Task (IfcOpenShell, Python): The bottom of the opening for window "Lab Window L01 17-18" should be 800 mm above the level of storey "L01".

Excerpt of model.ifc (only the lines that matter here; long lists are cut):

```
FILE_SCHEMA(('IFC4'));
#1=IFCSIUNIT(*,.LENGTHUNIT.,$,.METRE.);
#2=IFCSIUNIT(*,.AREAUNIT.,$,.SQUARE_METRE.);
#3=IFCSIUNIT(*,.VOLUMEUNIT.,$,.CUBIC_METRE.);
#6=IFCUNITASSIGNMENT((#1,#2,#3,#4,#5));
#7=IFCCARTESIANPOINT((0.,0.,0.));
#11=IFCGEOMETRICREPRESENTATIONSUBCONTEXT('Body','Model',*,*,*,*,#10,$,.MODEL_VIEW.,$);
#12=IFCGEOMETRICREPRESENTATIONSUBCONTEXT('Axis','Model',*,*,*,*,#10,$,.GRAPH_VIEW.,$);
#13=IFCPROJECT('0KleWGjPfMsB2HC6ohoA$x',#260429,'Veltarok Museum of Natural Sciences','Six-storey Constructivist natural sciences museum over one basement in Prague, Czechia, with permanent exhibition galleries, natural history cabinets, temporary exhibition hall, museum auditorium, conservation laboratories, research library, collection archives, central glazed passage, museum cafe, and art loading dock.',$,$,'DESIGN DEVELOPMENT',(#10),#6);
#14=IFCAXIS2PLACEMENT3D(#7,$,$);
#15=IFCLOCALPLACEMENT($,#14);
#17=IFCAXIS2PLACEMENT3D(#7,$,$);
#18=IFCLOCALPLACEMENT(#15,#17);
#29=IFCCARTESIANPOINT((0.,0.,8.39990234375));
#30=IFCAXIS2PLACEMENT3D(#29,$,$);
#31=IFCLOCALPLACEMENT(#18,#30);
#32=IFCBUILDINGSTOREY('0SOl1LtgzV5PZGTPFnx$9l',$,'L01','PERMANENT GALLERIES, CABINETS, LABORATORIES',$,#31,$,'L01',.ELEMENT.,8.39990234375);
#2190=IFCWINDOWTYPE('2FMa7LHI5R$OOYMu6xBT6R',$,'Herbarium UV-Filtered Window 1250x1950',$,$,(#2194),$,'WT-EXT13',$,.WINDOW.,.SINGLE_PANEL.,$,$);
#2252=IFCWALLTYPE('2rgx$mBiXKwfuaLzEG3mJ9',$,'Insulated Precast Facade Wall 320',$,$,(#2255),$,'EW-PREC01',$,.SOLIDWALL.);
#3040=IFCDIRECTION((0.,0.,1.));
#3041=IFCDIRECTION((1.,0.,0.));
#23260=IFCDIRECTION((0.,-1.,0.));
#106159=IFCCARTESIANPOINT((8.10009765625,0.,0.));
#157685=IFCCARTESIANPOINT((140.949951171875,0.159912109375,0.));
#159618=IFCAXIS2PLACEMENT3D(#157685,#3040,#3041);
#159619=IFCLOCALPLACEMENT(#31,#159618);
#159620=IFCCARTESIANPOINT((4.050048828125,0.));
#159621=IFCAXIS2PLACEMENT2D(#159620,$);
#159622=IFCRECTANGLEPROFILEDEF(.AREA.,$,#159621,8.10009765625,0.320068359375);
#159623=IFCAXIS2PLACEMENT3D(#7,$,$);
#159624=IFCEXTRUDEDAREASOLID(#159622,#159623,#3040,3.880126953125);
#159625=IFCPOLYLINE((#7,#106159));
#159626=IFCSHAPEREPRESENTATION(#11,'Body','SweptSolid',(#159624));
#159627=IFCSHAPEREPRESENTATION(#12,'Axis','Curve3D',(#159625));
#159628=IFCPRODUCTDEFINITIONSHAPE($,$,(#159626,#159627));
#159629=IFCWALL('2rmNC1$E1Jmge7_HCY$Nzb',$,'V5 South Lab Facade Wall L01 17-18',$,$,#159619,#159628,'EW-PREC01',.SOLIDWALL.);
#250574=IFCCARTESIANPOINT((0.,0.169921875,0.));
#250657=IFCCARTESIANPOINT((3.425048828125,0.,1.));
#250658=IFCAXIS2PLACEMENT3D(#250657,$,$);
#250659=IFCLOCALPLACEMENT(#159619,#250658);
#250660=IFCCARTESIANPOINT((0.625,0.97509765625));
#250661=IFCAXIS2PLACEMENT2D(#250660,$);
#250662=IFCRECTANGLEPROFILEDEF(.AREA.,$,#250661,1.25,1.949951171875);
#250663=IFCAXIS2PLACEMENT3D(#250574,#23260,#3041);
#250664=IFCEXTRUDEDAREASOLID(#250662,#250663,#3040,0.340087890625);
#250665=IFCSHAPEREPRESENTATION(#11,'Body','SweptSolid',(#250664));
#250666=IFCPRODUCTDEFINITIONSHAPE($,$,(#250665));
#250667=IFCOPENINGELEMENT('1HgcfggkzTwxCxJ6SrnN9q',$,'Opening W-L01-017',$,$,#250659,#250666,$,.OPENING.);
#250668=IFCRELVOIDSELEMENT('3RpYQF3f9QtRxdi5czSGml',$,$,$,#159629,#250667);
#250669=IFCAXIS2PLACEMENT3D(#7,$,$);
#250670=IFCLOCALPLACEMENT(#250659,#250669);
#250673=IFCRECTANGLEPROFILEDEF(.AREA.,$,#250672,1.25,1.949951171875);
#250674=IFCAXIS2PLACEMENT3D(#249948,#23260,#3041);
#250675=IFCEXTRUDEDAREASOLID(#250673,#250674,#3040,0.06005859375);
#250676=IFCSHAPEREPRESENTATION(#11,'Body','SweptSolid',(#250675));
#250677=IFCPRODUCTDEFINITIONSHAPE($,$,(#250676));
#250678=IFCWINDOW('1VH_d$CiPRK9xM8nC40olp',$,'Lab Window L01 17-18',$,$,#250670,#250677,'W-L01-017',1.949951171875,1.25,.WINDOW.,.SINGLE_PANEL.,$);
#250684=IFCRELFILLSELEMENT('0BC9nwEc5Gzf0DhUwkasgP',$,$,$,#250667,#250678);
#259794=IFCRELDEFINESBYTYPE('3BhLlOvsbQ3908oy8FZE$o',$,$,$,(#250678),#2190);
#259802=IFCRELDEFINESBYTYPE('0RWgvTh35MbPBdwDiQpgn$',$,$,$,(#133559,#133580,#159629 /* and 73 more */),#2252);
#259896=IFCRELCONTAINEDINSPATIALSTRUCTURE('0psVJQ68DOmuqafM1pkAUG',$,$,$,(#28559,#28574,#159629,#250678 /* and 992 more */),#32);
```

```python
import numpy as np
import ifcopenshell
import ifcopenshell.api.geometry
import ifcopenshell.geom
import ifcopenshell.util.element
import ifcopenshell.util.placement
import ifcopenshell.util.shape
import ifcopenshell.util.unit

model = ifcopenshell.open("model.ifc")
unit_scale = ifcopenshell.util.unit.calculate_unit_scale(model)

window = model.by_guid("1VH_d$CiPRK9xM8nC40olp")
opening = window.FillsVoids[0].RelatingOpeningElement
storey = ifcopenshell.util.element.get_container(window, ifc_class="IfcBuildingStorey")
level = ifcopenshell.util.placement.get_local_placement(storey.ObjectPlacement)[2, 3]

# The opening's origin need not be at the sill, so measure its lowest point.
shape = ifcopenshell.geom.create_shape(ifcopenshell.geom.settings(), opening)
bottom = ifcopenshell.util.shape.get_shape_bottom_elevation(shape, shape.geometry) / unit_scale
dz = level + 0.8 / unit_scale - bottom

shift = np.array([0.0, 0.0, dz])
# The window is placed relative to its opening, so it follows when the opening moves.
matrix = ifcopenshell.util.placement.get_local_placement(opening.ObjectPlacement)
matrix[:3, 3] += shift
ifcopenshell.api.geometry.edit_object_placement(
    model, product=opening, matrix=matrix, is_si=False, should_transform_children=True
)

print(f"moved by {dz * unit_scale:+.3f} m")

model.write("model_updated.ifc")
```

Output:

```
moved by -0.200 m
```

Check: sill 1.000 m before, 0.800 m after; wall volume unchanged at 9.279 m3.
